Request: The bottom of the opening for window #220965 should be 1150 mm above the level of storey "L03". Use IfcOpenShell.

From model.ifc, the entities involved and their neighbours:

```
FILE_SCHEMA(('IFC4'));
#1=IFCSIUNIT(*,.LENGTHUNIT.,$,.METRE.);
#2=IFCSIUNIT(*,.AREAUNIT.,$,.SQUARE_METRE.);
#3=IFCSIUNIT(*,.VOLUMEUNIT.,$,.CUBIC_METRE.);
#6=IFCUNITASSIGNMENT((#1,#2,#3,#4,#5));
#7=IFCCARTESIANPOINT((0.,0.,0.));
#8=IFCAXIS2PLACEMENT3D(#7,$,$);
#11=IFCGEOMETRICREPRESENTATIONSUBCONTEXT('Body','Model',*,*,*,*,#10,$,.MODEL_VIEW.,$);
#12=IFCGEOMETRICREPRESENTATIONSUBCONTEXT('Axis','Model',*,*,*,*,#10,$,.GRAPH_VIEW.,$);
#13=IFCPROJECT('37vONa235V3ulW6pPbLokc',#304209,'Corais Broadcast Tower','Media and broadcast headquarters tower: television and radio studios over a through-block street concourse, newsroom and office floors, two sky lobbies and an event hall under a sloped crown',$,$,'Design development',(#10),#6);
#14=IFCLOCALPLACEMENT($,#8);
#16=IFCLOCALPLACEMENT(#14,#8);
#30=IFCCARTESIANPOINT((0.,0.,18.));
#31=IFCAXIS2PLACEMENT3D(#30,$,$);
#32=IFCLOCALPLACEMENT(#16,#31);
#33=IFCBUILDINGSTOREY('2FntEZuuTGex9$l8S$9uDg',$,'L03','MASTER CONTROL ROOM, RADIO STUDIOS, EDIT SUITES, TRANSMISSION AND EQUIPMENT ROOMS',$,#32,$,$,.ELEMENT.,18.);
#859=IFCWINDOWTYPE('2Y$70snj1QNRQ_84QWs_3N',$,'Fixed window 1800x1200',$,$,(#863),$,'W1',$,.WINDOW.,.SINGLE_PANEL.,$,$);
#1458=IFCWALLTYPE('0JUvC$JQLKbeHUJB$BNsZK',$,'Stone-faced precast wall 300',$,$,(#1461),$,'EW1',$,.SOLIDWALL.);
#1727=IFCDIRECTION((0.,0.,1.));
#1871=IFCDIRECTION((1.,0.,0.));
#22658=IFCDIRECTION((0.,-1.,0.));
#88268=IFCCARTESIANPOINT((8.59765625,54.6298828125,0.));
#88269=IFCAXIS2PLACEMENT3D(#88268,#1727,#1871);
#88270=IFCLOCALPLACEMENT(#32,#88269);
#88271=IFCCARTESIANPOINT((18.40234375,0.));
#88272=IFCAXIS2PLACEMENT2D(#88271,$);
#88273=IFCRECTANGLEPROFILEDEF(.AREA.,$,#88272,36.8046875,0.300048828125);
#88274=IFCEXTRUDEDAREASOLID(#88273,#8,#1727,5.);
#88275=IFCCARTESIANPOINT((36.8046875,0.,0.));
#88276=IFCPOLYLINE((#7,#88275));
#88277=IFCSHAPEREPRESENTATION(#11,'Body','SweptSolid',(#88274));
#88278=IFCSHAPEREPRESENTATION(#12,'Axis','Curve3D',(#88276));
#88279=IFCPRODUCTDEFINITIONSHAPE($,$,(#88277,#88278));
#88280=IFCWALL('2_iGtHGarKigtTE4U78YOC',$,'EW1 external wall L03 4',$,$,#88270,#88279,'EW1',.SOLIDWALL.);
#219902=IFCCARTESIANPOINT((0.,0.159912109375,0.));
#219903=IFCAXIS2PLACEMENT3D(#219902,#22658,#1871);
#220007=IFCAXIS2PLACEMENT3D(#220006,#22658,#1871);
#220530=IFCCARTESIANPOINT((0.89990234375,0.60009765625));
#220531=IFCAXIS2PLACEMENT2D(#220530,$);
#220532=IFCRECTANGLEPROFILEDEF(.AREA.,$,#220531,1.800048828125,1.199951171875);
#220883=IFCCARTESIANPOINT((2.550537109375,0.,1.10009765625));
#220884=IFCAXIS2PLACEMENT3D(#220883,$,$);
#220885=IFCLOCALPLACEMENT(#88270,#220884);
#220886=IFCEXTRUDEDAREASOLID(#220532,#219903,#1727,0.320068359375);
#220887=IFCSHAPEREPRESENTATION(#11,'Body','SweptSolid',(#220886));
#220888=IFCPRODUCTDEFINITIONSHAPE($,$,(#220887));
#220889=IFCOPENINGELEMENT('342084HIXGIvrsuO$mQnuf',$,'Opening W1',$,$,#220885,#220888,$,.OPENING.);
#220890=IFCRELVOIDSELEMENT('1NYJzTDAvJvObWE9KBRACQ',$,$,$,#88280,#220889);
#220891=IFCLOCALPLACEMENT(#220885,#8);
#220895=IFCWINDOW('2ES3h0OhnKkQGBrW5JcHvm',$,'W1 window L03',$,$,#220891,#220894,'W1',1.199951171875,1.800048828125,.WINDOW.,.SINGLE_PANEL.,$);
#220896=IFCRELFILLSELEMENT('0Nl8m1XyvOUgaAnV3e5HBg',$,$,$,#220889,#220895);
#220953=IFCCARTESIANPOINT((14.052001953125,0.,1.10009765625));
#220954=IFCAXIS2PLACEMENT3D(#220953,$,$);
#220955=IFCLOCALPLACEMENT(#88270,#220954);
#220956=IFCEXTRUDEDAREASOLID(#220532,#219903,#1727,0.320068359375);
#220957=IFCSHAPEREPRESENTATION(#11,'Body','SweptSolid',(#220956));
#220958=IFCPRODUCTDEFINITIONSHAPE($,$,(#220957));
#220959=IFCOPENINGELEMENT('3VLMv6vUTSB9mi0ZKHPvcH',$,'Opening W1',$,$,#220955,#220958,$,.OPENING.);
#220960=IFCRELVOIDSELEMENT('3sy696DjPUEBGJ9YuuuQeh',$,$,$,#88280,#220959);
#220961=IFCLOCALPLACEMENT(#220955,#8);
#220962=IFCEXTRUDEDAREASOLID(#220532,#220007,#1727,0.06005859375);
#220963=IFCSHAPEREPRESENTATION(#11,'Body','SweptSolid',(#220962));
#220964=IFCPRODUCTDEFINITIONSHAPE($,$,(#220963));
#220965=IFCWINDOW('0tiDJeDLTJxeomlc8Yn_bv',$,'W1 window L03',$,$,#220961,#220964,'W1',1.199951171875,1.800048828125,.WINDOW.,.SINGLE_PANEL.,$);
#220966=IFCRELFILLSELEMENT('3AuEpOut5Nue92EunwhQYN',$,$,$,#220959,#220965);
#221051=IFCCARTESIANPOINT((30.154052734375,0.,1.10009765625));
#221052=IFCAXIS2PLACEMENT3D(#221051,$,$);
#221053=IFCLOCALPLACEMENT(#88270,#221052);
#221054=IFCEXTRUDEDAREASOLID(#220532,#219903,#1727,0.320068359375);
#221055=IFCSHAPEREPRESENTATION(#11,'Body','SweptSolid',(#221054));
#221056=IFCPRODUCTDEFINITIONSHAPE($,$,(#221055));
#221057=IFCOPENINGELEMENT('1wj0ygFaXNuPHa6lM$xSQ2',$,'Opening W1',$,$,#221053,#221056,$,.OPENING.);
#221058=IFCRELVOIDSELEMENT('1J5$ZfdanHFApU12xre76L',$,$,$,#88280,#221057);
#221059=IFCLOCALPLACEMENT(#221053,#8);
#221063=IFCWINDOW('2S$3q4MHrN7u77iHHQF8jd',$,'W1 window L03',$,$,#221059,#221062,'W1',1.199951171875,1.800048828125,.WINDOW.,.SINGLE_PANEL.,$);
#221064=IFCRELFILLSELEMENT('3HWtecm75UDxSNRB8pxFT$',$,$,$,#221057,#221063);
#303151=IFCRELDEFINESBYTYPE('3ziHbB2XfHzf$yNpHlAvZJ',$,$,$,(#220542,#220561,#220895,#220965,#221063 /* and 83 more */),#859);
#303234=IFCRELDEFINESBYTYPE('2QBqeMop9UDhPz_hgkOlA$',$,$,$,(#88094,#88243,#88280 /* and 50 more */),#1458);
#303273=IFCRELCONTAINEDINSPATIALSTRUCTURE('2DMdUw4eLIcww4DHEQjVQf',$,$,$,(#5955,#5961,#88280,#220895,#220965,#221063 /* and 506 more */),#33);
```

```python
import numpy as np
import ifcopenshell
import ifcopenshell.api.geometry
import ifcopenshell.geom
import ifcopenshell.util.element
import ifcopenshell.util.placement
import ifcopenshell.util.shape
import ifcopenshell.util.unit

model = ifcopenshell.open("model.ifc")
unit_scale = ifcopenshell.util.unit.calculate_unit_scale(model)

window = model.by_guid("0tiDJeDLTJxeomlc8Yn_bv")
opening = window.FillsVoids[0].RelatingOpeningElement
storey = ifcopenshell.util.element.get_container(window, ifc_class="IfcBuildingStorey")
level = ifcopenshell.util.placement.get_local_placement(storey.ObjectPlacement)[2, 3]

# The opening's origin need not be at the sill, so measure its lowest point.
shape = ifcopenshell.geom.create_shape(ifcopenshell.geom.settings(), opening)
bottom = ifcopenshell.util.shape.get_shape_bottom_elevation(shape, shape.geometry) / unit_scale
dz = level + 1.15 - bottom

shift = np.array([0.0, 0.0, dz])
# The window is placed relative to its opening, so it follows when the opening moves.
matrix = ifcopenshell.util.placement.get_local_placement(opening.ObjectPlacement)
matrix[:3, 3] += shift
ifcopenshell.api.geometry.edit_object_placement(
    model, product=opening, matrix=matrix, is_si=False, should_transform_children=True
)

print(f"moved by {dz * unit_scale:+.3f} m")

model.write("model_updated.ifc")
```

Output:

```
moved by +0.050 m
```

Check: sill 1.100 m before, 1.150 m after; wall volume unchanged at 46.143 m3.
